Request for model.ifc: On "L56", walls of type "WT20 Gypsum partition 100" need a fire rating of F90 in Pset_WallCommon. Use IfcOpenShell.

First a look at what the model holds.

```python
import ifcopenshell
import ifcopenshell.util.element

model = ifcopenshell.open("model.ifc")
print(model.schema)
storey = next(s for s in model.by_type("IfcBuildingStorey") if s.Name == "L56")
walls = [e for e in ifcopenshell.util.element.get_decomposition(storey) if e.is_a("IfcWall")]
seen = {}
for e in walls:
    element_type = ifcopenshell.util.element.get_type(e)
    key = (element_type.Name if element_type != e and element_type else None, ifcopenshell.util.element.get_pset(e, "Pset_WallCommon", "FireRating"))
    seen[key] = seen.get(key, 0) + 1
for (name, value), count in sorted(seen.items(), key=str):
    print(count, "x", name, "|", value)
```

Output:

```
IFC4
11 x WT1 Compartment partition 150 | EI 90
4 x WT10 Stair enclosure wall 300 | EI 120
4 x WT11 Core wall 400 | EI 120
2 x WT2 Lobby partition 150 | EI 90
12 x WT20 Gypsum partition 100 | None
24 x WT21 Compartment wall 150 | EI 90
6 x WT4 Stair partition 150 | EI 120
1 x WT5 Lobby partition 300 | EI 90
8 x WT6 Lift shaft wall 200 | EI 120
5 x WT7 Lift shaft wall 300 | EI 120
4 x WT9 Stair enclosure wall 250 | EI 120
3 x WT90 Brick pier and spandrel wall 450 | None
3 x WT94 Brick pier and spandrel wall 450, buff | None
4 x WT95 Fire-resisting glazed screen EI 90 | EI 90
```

```python
import ifcopenshell
import ifcopenshell.api.pset
import ifcopenshell.util.element

model = ifcopenshell.open("model.ifc")

storey = next(s for s in model.by_type("IfcBuildingStorey") if s.Name == "L56")
walls = [e for e in ifcopenshell.util.element.get_decomposition(storey) if e.is_a("IfcWall")]

count = 0
for e in walls:
    element_type = ifcopenshell.util.element.get_type(e)
    if element_type in (None, e) or element_type.Name != "WT20 Gypsum partition 100":
        continue
    found = ifcopenshell.util.element.get_pset(e, "Pset_WallCommon", should_inherit=False)
    if found:
        pset = model.by_id(found["id"])
        if len(ifcopenshell.util.element.get_elements_by_pset(pset)) > 1:
            pset = ifcopenshell.api.pset.unshare_pset(model, products=[e], pset=pset)[0]
    else:
        pset = ifcopenshell.api.pset.add_pset(model, product=e, name="Pset_WallCommon")
    ifcopenshell.api.pset.edit_pset(model, pset=pset, properties={"FireRating": "F90"})
    count += 1

print(count, "walls updated")

model.write("model_v2.ifc")
```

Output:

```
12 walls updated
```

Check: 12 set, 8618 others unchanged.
